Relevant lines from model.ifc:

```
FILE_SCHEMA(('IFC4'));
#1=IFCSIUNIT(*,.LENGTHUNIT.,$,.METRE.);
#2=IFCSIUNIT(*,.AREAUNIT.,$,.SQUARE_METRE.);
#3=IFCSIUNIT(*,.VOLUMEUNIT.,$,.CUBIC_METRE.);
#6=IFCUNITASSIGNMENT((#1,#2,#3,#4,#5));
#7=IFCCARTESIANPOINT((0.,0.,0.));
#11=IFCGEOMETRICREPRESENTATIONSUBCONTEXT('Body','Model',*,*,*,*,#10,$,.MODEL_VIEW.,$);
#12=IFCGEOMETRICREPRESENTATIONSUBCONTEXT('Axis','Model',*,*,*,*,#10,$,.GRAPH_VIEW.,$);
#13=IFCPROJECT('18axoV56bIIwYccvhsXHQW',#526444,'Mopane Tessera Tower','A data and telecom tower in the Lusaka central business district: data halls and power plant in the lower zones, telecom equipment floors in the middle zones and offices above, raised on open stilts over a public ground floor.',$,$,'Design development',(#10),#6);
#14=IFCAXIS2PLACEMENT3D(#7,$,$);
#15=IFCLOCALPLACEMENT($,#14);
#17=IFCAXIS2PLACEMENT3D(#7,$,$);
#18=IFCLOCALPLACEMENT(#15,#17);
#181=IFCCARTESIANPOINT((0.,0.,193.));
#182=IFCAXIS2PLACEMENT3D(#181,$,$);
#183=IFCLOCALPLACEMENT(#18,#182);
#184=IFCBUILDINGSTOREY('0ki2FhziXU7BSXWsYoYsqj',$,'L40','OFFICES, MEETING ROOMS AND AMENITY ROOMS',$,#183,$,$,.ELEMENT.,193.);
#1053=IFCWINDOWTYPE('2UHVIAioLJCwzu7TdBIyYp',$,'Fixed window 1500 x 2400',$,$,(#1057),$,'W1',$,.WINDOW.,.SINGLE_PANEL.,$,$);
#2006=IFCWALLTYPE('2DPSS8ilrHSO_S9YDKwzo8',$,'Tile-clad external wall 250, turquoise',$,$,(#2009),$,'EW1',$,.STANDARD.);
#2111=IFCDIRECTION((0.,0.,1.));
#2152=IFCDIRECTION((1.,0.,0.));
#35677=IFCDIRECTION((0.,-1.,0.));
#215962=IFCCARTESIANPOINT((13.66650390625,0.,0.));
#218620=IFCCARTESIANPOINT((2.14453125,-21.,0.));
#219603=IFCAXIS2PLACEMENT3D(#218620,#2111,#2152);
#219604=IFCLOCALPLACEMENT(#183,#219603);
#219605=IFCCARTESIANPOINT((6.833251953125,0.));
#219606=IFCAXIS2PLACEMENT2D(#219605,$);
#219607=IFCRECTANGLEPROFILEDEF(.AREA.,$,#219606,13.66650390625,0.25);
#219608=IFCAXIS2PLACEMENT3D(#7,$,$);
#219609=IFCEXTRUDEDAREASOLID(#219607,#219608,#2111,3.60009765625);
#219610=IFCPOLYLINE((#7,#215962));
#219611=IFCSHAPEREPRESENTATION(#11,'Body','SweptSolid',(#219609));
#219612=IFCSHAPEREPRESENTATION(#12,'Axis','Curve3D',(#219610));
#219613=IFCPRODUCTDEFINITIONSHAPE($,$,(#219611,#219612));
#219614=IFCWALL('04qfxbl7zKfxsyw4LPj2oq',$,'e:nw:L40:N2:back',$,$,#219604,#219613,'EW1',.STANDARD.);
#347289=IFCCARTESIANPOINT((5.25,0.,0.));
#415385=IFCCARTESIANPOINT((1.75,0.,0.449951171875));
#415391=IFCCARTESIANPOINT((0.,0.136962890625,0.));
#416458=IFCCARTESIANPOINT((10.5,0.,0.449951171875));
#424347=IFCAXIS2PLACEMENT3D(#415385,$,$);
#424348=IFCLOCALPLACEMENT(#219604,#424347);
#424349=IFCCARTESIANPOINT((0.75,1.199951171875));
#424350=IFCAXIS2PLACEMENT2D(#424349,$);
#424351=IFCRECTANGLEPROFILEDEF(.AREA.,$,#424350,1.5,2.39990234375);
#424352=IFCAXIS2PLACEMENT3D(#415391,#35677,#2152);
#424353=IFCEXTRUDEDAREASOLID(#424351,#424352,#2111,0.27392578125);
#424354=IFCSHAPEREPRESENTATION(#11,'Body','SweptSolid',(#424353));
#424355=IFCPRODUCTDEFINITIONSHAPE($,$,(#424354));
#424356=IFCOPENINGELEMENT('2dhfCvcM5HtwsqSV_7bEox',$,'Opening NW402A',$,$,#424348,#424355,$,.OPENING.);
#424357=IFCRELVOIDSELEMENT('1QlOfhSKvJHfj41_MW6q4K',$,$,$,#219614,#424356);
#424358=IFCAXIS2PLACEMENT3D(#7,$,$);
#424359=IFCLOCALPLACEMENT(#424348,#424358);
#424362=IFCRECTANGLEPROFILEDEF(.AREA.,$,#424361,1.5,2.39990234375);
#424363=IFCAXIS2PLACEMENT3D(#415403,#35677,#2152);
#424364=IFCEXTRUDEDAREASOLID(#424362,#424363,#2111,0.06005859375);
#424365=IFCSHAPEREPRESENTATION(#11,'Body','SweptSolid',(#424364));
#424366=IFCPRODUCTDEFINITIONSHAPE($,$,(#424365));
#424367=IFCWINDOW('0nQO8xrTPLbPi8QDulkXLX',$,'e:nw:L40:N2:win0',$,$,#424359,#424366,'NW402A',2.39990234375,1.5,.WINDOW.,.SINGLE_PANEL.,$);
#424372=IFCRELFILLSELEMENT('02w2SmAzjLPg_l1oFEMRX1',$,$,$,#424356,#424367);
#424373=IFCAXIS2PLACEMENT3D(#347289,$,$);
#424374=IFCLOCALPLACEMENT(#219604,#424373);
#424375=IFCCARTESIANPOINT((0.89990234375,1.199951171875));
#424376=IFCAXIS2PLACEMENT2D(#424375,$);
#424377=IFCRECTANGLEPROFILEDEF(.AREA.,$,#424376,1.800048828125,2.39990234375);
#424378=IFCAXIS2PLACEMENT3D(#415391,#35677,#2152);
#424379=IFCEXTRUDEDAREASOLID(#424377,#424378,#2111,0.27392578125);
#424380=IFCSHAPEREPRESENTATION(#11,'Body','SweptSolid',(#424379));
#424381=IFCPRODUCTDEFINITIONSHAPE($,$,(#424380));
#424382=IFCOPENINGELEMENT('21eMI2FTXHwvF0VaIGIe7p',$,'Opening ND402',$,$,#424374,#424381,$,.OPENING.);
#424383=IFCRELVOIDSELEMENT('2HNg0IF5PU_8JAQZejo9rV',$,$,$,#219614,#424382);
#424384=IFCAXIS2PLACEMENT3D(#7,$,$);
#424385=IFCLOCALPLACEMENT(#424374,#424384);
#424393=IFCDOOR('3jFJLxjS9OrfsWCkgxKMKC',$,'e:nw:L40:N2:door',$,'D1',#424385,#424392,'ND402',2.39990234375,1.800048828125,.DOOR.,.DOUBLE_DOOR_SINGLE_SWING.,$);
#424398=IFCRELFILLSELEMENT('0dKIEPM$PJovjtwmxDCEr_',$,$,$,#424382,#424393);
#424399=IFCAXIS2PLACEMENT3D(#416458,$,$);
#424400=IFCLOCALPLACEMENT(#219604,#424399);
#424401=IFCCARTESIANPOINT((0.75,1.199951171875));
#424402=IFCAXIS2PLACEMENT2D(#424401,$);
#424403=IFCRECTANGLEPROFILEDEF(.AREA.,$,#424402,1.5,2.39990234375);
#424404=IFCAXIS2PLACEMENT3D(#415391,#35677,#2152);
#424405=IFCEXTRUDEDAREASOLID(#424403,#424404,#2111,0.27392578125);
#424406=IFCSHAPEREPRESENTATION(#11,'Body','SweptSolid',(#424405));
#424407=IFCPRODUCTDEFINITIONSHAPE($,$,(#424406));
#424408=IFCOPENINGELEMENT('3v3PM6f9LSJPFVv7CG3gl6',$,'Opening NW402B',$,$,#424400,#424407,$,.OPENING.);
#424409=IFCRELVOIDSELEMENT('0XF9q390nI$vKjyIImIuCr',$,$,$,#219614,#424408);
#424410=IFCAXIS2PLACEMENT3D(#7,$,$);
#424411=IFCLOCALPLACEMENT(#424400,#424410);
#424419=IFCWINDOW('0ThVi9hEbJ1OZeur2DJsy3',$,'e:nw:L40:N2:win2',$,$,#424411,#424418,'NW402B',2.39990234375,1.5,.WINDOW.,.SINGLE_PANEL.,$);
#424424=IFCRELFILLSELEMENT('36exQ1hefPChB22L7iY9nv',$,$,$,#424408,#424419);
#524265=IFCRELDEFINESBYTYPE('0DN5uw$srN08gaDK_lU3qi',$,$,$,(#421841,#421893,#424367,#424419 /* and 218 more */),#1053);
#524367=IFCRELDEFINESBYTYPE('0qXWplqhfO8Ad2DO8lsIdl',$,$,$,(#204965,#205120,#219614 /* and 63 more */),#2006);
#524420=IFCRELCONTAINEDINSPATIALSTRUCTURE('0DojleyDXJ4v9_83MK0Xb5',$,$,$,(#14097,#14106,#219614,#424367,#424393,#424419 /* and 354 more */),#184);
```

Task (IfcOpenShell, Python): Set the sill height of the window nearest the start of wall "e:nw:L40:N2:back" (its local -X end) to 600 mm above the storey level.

```python
import numpy as np
import ifcopenshell
import ifcopenshell.api.geometry
import ifcopenshell.geom
import ifcopenshell.util.element
import ifcopenshell.util.placement
import ifcopenshell.util.shape
import ifcopenshell.util.unit

model = ifcopenshell.open("model.ifc")
unit_scale = ifcopenshell.util.unit.calculate_unit_scale(model)

window = model.by_id(424367)
opening = window.FillsVoids[0].RelatingOpeningElement
storey = ifcopenshell.util.element.get_container(window, ifc_class="IfcBuildingStorey")
level = ifcopenshell.util.placement.get_local_placement(storey.ObjectPlacement)[2, 3]

# The opening's origin need not be at the sill, so measure its lowest point.
shape = ifcopenshell.geom.create_shape(ifcopenshell.geom.settings(), opening)
bottom = ifcopenshell.util.shape.get_shape_bottom_elevation(shape, shape.geometry) / unit_scale
dz = level + 0.6 / unit_scale - bottom

shift = np.array([0.0, 0.0, dz])
# The window is placed relative to its opening, so it follows when the opening moves.
matrix = ifcopenshell.util.placement.get_local_placement(opening.ObjectPlacement)
matrix[:3, 3] += shift
ifcopenshell.api.geometry.edit_object_placement(
    model, product=opening, matrix=matrix, is_si=False, should_transform_children=True
)

print(f"moved by {dz * unit_scale:+.3f} m")

model.write("model_v2.ifc")
```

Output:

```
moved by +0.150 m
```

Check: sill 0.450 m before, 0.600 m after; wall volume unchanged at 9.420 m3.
